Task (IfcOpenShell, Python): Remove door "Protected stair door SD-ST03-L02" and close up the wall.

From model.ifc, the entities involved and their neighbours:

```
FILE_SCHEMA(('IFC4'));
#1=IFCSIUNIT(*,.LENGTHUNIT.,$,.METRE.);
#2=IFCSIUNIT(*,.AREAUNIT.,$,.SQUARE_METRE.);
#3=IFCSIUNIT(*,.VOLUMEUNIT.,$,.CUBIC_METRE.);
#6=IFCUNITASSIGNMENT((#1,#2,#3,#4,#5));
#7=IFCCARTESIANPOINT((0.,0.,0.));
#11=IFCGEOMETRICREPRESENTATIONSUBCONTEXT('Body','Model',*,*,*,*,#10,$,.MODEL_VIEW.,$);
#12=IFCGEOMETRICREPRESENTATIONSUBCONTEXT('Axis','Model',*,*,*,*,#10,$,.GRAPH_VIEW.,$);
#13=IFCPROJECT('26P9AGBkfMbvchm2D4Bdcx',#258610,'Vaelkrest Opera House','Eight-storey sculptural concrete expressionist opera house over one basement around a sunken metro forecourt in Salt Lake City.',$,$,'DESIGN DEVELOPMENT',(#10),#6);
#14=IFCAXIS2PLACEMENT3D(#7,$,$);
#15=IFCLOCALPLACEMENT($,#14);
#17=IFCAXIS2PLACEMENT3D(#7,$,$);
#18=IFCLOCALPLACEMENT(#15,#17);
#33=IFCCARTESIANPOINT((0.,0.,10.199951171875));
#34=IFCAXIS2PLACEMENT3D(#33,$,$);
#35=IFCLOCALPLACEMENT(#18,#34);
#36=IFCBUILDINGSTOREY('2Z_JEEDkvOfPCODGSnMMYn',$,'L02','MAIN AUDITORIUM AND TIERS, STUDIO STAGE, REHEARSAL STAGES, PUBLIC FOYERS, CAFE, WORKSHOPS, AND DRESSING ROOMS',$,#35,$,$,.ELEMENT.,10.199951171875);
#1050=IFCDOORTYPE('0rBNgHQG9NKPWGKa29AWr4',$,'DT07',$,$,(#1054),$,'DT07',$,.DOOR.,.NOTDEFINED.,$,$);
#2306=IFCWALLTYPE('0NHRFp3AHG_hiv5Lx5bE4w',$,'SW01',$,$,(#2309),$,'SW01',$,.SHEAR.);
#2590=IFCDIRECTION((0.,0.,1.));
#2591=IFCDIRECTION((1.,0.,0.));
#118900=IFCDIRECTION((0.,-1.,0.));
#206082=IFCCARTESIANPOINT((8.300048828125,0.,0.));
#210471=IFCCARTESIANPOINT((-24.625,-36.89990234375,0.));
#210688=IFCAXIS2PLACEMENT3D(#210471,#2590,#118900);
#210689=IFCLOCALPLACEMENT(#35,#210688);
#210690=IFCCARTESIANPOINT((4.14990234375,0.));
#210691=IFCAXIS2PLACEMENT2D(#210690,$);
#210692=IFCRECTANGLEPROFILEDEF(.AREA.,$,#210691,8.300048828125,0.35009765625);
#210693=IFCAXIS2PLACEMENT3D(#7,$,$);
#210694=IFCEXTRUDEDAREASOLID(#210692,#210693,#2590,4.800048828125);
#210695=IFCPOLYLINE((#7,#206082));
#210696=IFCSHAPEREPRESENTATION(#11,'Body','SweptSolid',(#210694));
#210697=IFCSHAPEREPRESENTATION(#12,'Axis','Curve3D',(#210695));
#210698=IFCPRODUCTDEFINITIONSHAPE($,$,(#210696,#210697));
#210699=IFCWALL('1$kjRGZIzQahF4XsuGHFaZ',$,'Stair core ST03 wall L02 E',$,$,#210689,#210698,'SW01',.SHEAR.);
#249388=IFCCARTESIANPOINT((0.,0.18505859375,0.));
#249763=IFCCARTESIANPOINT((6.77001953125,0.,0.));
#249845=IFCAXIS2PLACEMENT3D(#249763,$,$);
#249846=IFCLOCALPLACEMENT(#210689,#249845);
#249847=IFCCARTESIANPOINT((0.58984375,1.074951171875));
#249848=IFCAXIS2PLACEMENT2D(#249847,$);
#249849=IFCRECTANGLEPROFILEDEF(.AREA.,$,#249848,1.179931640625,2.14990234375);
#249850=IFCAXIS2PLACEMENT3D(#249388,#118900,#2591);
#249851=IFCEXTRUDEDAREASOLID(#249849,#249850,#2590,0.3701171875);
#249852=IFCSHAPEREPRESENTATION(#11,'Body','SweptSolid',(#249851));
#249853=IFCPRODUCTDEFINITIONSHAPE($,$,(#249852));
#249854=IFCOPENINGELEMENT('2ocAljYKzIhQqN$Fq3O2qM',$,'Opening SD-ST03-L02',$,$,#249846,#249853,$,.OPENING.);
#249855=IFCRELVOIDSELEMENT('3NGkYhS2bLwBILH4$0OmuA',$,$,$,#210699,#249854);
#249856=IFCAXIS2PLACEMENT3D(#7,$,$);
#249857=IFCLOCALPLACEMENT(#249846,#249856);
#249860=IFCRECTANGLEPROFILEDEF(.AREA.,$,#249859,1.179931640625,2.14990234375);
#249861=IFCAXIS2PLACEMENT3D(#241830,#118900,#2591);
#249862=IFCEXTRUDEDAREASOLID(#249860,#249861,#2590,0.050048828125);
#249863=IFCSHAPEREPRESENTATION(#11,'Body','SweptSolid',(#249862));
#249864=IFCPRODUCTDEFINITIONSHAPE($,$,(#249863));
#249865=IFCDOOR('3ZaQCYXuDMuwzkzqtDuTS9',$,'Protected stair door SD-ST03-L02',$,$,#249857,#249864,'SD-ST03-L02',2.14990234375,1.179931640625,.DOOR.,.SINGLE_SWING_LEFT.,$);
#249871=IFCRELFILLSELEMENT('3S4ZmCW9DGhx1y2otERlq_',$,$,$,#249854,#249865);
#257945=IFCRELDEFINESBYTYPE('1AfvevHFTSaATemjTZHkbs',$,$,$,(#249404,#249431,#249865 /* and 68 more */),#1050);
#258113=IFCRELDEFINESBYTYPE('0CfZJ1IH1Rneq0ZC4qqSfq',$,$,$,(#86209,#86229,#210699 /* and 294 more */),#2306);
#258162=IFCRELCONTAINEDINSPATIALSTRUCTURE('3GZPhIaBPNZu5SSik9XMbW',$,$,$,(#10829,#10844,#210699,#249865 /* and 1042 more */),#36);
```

```python
import ifcopenshell
import ifcopenshell.api.feature
import ifcopenshell.api.root
import ifcopenshell.geom
import ifcopenshell.util.shape

model = ifcopenshell.open("model.ifc")
settings = ifcopenshell.geom.settings()


def volume(element):
    """Net volume in cubic metres, openings subtracted."""
    shape = ifcopenshell.geom.create_shape(settings, element)
    return ifcopenshell.util.shape.get_volume(shape.geometry)


door = model.by_guid("3ZaQCYXuDMuwzkzqtDuTS9")
opening = door.FillsVoids[0].RelatingOpeningElement
wall = opening.VoidsElements[0].RelatingBuildingElement
before = volume(wall)

ifcopenshell.api.root.remove_product(model, product=door)
ifcopenshell.api.feature.remove_feature(model, feature=opening)

after = volume(wall)

print(f"wall volume {before:.3f} -> {after:.3f} m3")

model.write("model-out.ifc")
```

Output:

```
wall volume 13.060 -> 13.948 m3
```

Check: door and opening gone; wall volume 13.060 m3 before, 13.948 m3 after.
